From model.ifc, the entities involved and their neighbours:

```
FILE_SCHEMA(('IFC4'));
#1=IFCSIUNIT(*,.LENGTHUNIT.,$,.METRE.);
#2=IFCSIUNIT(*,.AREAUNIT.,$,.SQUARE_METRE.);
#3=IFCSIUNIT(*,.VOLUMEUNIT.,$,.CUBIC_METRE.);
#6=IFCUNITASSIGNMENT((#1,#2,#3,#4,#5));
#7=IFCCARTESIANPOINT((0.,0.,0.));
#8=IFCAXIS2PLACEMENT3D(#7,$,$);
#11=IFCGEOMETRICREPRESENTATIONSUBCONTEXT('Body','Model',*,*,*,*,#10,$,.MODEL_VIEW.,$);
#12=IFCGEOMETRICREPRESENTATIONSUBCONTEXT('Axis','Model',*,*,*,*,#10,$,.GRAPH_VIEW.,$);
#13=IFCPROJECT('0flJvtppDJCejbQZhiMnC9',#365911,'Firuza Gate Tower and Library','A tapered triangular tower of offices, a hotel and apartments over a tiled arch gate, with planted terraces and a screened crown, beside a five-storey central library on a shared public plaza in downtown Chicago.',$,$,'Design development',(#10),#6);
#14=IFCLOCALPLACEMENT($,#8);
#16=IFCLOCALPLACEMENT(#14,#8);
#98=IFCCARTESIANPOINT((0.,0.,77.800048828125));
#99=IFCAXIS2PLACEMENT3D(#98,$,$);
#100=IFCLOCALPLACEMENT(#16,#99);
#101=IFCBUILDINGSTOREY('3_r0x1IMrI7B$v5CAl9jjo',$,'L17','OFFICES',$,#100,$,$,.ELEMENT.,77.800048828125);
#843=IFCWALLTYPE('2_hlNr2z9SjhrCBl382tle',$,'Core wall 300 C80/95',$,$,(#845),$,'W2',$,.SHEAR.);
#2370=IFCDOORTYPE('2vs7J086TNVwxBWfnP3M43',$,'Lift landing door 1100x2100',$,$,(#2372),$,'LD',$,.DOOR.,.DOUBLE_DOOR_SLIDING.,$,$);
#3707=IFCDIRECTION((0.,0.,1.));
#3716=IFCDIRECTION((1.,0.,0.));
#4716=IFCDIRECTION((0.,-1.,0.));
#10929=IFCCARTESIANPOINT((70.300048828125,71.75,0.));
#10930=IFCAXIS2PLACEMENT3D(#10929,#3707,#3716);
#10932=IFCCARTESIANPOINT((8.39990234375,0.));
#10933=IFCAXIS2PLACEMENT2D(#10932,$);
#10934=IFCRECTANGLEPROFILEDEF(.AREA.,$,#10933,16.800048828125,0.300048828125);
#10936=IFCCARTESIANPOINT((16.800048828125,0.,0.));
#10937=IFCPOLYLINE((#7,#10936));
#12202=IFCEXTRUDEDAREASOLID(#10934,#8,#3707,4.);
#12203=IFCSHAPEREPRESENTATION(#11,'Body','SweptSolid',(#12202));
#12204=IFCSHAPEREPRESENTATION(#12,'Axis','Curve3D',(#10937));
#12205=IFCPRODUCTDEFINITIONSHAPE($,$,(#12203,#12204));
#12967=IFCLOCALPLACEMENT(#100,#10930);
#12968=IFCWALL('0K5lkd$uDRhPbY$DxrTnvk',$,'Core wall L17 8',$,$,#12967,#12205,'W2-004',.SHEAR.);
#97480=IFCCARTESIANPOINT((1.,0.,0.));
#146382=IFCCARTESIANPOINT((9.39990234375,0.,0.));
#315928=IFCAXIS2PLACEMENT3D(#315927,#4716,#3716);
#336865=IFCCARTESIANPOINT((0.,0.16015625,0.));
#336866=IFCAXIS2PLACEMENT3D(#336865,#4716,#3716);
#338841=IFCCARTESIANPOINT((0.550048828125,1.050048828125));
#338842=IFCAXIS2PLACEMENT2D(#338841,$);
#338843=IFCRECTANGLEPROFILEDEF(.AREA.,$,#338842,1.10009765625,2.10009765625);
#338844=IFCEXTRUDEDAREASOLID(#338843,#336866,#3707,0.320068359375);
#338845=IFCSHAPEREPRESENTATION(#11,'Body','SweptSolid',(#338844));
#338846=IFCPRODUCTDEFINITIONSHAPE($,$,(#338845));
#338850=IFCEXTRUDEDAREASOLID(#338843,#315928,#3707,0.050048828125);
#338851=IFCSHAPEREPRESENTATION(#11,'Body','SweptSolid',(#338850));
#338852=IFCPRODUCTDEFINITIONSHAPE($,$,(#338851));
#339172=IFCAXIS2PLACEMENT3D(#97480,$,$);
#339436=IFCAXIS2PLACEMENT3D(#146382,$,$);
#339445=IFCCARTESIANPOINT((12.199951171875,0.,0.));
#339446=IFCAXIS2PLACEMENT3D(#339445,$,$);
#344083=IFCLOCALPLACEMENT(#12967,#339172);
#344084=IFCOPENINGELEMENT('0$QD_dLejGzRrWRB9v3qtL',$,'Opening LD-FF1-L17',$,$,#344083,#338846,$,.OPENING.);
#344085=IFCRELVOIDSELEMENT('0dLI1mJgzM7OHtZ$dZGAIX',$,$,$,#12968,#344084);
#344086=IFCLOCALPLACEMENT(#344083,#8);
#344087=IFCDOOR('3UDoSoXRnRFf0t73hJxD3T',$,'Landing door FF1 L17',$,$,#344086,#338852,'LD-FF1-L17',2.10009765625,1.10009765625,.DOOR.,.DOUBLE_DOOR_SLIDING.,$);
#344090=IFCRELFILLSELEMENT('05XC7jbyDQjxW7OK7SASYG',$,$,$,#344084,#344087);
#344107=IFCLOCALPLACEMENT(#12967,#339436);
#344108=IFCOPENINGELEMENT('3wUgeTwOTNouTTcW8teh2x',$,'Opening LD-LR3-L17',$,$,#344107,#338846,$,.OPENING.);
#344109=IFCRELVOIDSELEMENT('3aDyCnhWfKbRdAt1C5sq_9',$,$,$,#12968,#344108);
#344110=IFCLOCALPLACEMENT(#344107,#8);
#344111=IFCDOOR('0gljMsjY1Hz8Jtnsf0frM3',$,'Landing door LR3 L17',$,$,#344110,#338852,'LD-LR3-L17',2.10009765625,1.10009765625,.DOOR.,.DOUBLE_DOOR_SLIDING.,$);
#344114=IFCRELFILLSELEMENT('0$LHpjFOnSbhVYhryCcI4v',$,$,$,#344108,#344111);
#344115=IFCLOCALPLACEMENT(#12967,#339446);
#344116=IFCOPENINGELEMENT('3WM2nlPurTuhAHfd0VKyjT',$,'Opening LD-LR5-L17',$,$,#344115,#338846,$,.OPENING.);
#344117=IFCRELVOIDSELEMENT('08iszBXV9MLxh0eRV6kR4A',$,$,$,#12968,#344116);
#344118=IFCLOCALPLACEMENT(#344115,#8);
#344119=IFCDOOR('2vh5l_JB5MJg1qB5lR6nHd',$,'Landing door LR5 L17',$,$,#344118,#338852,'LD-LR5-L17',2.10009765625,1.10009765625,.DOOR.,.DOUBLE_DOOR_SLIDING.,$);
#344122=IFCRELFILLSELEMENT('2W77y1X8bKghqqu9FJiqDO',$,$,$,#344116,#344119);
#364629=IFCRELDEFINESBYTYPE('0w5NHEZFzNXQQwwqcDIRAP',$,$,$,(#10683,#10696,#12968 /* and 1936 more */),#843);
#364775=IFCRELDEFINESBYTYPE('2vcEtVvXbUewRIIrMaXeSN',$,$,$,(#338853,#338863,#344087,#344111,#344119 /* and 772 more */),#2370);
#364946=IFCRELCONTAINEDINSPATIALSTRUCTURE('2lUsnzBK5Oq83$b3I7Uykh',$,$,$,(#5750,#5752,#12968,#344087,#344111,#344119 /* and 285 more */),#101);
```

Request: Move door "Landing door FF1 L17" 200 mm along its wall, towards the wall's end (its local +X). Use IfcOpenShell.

```python
import ifcopenshell
import ifcopenshell.api.geometry
import ifcopenshell.util.placement
import ifcopenshell.util.unit

model = ifcopenshell.open("model.ifc")
unit_scale = ifcopenshell.util.unit.calculate_unit_scale(model)

door = model.by_guid("3UDoSoXRnRFf0t73hJxD3T")
opening = door.FillsVoids[0].RelatingOpeningElement
wall = opening.VoidsElements[0].RelatingBuildingElement

wall_matrix = ifcopenshell.util.placement.get_local_placement(wall.ObjectPlacement)
shift = wall_matrix[:3, 0] * 0.2 / unit_scale
before = ifcopenshell.util.placement.get_local_placement(door.ObjectPlacement)[:3, 3].copy()

# The door is placed relative to its opening, so it follows when the opening moves.
matrix = ifcopenshell.util.placement.get_local_placement(opening.ObjectPlacement)
matrix[:3, 3] += shift
ifcopenshell.api.geometry.edit_object_placement(
    model, product=opening, matrix=matrix, is_si=False, should_transform_children=True
)

after = ifcopenshell.util.placement.get_local_placement(door.ObjectPlacement)[:3, 3]
print("door moved by", (after - before).round(3) + 0.0)

model.write("model_rev.ifc")
```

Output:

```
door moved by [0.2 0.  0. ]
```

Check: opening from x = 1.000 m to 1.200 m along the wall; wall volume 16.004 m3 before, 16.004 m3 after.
